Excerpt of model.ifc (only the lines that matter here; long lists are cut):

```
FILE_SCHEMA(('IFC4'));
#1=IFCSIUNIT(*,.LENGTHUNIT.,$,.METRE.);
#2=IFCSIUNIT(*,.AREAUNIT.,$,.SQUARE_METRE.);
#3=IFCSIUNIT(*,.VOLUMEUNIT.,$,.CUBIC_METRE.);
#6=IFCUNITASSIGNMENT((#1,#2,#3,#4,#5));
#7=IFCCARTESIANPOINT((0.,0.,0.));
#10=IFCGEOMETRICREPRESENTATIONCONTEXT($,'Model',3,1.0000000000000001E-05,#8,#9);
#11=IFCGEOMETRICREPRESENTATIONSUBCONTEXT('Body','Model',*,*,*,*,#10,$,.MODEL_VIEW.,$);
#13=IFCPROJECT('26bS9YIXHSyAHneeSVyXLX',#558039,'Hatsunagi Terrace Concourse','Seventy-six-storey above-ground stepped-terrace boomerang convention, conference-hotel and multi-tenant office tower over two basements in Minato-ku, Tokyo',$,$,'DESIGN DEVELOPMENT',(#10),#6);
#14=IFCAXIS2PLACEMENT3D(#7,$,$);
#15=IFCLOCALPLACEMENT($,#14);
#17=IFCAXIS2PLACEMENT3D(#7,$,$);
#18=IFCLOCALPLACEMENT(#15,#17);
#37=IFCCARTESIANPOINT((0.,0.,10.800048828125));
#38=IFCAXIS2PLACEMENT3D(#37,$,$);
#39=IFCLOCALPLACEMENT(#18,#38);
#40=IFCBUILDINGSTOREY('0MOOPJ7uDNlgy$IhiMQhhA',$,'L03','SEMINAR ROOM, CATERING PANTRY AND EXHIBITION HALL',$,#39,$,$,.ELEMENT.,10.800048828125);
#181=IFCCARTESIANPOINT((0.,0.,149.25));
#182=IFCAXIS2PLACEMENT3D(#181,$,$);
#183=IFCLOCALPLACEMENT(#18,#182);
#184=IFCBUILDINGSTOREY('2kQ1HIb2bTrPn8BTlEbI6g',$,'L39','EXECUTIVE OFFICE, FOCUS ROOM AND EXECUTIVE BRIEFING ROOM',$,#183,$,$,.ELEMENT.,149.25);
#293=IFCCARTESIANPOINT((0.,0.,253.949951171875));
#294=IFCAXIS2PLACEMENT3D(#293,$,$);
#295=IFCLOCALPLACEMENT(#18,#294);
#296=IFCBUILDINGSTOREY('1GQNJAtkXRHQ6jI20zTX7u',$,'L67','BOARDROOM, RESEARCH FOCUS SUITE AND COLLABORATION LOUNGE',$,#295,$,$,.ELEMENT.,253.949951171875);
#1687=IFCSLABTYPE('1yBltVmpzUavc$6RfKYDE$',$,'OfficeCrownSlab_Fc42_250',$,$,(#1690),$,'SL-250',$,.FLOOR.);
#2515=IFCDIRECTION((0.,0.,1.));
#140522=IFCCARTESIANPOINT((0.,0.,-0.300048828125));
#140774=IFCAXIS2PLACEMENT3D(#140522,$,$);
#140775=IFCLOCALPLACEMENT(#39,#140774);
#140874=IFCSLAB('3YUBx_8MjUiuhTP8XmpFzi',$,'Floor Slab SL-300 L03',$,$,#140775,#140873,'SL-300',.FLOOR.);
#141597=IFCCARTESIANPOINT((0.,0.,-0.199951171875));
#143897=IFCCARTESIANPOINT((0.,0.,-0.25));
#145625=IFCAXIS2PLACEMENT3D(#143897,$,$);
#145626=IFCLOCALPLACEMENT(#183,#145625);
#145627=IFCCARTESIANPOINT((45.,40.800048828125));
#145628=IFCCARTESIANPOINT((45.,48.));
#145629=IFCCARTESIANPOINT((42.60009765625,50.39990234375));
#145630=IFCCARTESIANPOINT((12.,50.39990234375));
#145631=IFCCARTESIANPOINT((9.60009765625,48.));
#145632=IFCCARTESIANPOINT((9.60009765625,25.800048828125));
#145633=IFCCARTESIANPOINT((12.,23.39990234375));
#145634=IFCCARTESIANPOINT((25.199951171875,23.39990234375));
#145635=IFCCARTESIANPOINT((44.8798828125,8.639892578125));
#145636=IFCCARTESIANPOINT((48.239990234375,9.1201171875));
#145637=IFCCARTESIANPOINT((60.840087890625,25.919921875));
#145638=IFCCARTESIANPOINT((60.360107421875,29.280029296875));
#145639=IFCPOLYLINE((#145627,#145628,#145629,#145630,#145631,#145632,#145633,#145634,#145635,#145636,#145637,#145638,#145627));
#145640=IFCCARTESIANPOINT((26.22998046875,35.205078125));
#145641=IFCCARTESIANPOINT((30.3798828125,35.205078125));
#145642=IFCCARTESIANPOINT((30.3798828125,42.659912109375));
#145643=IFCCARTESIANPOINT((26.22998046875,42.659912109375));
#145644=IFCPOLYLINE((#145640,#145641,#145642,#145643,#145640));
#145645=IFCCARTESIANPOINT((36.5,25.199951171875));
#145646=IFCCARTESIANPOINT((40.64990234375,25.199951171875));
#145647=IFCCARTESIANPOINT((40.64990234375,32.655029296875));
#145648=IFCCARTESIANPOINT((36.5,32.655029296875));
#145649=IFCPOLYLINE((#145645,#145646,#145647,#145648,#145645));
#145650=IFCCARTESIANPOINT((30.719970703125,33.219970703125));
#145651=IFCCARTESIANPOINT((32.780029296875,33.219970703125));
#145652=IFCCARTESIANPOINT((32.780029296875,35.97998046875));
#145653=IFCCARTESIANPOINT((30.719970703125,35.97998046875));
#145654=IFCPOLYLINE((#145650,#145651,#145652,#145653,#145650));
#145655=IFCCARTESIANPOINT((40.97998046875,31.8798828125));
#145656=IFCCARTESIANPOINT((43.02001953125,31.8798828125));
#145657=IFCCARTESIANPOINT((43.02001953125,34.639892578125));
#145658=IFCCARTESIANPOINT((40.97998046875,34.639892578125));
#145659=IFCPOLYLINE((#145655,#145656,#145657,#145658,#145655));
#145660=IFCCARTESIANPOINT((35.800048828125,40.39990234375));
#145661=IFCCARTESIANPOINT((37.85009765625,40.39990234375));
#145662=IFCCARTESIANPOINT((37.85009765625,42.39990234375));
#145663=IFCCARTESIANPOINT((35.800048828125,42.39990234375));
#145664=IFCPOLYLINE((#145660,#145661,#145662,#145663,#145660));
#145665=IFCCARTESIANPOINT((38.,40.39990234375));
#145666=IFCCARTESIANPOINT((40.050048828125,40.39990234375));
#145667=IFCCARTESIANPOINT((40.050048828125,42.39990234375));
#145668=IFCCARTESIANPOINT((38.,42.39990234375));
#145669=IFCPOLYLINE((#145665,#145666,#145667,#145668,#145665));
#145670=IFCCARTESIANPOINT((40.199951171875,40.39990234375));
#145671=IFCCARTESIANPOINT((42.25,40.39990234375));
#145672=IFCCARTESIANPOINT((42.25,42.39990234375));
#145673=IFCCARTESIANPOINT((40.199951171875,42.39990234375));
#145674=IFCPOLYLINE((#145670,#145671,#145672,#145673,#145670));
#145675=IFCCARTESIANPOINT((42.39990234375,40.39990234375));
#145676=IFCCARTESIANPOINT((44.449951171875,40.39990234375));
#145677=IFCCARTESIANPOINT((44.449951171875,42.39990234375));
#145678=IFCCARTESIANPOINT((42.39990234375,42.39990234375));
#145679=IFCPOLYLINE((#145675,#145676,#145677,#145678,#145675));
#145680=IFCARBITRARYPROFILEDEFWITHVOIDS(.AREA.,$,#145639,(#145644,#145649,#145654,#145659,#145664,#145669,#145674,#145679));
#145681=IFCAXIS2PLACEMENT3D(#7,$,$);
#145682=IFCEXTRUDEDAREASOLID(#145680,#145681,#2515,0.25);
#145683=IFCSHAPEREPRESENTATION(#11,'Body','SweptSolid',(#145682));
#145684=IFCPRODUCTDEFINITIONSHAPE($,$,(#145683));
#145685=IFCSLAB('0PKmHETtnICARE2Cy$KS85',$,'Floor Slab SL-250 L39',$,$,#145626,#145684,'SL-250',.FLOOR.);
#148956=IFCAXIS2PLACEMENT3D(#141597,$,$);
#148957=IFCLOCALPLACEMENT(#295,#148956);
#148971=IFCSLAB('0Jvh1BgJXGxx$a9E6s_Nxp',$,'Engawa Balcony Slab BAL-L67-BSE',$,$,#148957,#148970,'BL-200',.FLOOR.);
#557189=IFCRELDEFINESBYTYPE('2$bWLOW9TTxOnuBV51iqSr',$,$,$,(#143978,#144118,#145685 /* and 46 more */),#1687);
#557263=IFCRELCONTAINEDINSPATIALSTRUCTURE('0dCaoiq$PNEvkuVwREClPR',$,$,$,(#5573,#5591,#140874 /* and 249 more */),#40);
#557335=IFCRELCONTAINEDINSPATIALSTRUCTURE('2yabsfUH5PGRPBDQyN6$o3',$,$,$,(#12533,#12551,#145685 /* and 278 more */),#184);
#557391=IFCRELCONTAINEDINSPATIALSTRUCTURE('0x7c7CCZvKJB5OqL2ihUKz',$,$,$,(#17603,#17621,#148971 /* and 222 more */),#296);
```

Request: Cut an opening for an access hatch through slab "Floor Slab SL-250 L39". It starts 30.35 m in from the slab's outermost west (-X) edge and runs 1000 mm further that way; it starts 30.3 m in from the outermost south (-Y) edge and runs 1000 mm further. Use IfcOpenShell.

```python
import numpy as np
import ifcopenshell
import ifcopenshell.api.feature
import ifcopenshell.api.geometry
import ifcopenshell.api.root
import ifcopenshell.geom
import ifcopenshell.util.placement
import ifcopenshell.util.representation
import ifcopenshell.util.shape
import ifcopenshell.util.unit

model = ifcopenshell.open("model.ifc")
unit_scale = ifcopenshell.util.unit.calculate_unit_scale(model)
settings = ifcopenshell.geom.settings()


def volume(element):
    """Net volume in cubic metres, openings subtracted."""
    shape = ifcopenshell.geom.create_shape(settings, element)
    return ifcopenshell.util.shape.get_volume(shape.geometry)


slab = model.by_id(145685)
before = volume(slab)

# Extent in the slab's own axes, in metres. The edges named are its -X and -Y sides.
slab_shape = ifcopenshell.geom.create_shape(settings, slab)
vertices = ifcopenshell.util.shape.get_vertices(slab_shape.geometry)
x_min, y_min, bottom = vertices.min(axis=0)
top = vertices[:, 2].max()

opening = ifcopenshell.api.root.create_entity(model, ifc_class="IfcOpeningElement", name="Access hatch opening", predefined_type="OPENING")
context = ifcopenshell.util.representation.get_context(model, "Model", "Body", "MODEL_VIEW")
width, depth = 1, 1
outline = [(0.0, 0.0), (width, 0.0), (width, depth), (0.0, depth), (0.0, 0.0)]
# Overshoot both faces by 50 mm so the cut is clean.
shape = ifcopenshell.api.geometry.add_slab_representation(
    model, context=context, depth=top - bottom + 0.1, polyline=outline
)
ifcopenshell.api.geometry.assign_representation(model, product=opening, representation=shape)

matrix = ifcopenshell.util.placement.get_local_placement(slab.ObjectPlacement)
matrix[:, 3] = matrix @ np.append(np.array([x_min + 30.35, y_min + 30.3, bottom - 0.05]) / unit_scale, 1.0)
ifcopenshell.api.geometry.edit_object_placement(model, product=opening, matrix=matrix, is_si=False)
ifcopenshell.api.feature.add_feature(model, feature=opening, element=slab)

after = volume(slab)

print(f"slab volume {before:.3f} -> {after:.3f} m3")

model.write("model-out.ifc")
```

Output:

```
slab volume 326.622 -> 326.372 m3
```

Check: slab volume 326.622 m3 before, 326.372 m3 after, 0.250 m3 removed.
